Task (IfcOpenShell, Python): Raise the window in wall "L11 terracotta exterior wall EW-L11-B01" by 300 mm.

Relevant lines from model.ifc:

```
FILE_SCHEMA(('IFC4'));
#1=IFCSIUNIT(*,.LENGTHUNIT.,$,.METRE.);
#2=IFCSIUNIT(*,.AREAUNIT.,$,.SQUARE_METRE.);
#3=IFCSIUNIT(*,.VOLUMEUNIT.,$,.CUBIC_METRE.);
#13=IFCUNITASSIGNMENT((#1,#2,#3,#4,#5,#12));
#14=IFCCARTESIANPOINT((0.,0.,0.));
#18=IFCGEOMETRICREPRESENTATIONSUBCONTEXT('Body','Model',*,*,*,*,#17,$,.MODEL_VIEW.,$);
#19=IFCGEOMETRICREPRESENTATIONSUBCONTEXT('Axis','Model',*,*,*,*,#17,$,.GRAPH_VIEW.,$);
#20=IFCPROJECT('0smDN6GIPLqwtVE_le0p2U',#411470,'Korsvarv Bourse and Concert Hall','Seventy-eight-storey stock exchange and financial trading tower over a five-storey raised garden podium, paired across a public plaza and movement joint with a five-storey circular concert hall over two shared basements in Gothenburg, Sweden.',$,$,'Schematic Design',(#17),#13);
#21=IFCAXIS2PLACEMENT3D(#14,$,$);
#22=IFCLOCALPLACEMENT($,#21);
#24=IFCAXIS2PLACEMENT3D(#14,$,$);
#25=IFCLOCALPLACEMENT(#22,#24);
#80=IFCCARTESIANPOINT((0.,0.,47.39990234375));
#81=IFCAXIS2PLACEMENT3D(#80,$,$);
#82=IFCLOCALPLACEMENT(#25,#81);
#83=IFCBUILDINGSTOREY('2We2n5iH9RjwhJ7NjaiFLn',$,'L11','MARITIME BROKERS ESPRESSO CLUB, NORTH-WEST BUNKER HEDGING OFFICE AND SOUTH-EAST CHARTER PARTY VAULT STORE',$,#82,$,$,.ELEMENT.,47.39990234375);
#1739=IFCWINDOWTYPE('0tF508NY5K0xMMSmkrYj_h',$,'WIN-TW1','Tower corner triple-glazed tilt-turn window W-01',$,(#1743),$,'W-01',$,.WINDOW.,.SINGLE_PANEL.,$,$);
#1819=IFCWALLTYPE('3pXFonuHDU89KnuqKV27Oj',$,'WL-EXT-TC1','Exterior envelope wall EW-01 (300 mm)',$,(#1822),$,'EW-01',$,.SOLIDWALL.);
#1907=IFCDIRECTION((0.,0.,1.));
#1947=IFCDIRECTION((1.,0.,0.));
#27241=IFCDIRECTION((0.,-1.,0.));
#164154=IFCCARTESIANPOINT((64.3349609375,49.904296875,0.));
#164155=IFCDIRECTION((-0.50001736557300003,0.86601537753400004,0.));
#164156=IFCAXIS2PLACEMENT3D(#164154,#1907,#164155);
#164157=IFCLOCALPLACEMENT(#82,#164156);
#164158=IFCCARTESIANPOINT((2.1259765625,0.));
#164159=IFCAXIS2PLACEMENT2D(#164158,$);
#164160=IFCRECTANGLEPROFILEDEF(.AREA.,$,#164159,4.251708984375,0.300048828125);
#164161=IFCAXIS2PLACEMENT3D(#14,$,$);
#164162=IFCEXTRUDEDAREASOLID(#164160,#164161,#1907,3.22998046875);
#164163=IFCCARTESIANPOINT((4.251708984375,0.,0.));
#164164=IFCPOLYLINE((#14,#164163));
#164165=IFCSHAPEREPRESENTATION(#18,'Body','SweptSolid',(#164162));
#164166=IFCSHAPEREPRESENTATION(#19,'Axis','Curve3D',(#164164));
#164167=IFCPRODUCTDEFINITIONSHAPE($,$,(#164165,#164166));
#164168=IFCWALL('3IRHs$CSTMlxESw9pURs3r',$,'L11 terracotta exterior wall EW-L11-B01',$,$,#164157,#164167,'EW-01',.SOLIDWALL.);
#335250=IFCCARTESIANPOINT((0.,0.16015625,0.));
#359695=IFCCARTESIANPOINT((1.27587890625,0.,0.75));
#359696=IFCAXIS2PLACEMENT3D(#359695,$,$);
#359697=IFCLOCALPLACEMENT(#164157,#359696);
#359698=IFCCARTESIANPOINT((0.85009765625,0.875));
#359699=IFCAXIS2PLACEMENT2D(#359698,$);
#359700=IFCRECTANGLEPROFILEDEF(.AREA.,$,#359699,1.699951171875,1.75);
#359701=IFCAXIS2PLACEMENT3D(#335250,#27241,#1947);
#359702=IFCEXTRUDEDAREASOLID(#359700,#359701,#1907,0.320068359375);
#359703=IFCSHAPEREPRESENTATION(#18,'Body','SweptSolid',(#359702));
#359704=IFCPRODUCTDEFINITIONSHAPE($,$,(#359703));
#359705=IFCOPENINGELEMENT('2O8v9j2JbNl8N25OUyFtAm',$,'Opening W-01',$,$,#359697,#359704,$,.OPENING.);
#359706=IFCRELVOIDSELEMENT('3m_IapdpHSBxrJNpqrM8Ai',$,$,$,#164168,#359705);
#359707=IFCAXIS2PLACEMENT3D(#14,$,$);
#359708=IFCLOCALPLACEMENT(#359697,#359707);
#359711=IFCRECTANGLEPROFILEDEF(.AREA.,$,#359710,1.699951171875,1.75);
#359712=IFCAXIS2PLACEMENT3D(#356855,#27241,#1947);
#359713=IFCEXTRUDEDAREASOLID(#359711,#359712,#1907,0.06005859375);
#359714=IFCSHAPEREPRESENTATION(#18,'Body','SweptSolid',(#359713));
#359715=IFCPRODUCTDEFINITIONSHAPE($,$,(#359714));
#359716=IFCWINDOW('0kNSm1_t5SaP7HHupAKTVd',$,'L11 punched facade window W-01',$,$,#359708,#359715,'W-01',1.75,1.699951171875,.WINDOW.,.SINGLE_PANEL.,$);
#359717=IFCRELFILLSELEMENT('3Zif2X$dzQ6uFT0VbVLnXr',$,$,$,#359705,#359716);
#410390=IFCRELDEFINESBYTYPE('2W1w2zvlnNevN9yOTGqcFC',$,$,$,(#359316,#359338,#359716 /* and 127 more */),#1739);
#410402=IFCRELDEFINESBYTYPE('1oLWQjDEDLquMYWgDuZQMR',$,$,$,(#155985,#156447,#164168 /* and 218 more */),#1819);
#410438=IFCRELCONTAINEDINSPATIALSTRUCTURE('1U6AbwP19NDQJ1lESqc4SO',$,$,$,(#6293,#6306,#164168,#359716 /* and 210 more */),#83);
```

```python
import numpy as np
import ifcopenshell
import ifcopenshell.api.geometry
import ifcopenshell.util.placement
import ifcopenshell.util.unit

model = ifcopenshell.open("model.ifc")
unit_scale = ifcopenshell.util.unit.calculate_unit_scale(model)

window = model.by_guid("0kNSm1_t5SaP7HHupAKTVd")
opening = window.FillsVoids[0].RelatingOpeningElement
dz = 0.3 / unit_scale

shift = np.array([0.0, 0.0, dz])
# The window is placed relative to its opening, so it follows when the opening moves.
matrix = ifcopenshell.util.placement.get_local_placement(opening.ObjectPlacement)
matrix[:3, 3] += shift
ifcopenshell.api.geometry.edit_object_placement(
    model, product=opening, matrix=matrix, is_si=False, should_transform_children=True
)

print(f"moved by {dz * unit_scale:+.3f} m")

model.write("model_rev.ifc")
```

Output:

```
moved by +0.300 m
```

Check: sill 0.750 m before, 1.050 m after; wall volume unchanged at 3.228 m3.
